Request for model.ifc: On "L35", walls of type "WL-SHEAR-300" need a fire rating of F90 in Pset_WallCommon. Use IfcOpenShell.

First a look at what the model holds.

```python
import ifcopenshell
import ifcopenshell.util.element

model = ifcopenshell.open("model.ifc")
print(model.schema)
storey = next(s for s in model.by_type("IfcBuildingStorey") if s.Name == "L35")
walls = [e for e in ifcopenshell.util.element.get_decomposition(storey) if e.is_a("IfcWall")]
seen = {}
for e in walls:
    element_type = ifcopenshell.util.element.get_type(e)
    key = (element_type.Name if element_type != e and element_type else None, ifcopenshell.util.element.get_pset(e, "Pset_WallCommon", "FireRating"))
    seen[key] = seen.get(key, 0) + 1
for (name, value), count in sorted(seen.items(), key=str):
    print(count, "x", name, "|", value)
```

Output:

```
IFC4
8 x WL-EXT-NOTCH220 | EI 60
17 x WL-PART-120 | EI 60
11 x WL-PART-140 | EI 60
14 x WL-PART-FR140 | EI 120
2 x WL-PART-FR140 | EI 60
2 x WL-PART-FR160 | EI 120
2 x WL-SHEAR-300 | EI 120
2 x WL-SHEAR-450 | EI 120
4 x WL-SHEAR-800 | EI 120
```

```python
import ifcopenshell
import ifcopenshell.api.pset
import ifcopenshell.util.element

model = ifcopenshell.open("model.ifc")

storey = next(s for s in model.by_type("IfcBuildingStorey") if s.Name == "L35")
walls = [e for e in ifcopenshell.util.element.get_decomposition(storey) if e.is_a("IfcWall")]

count = 0
for e in walls:
    element_type = ifcopenshell.util.element.get_type(e)
    if element_type in (None, e) or element_type.Name != "WL-SHEAR-300":
        continue
    # add_pset returns the element's existing set when there is one.
    pset = ifcopenshell.api.pset.add_pset(model, product=e, name="Pset_WallCommon")
    ifcopenshell.api.pset.edit_pset(model, pset=pset, properties={"FireRating": "F90"})
    count += 1

print(count, "walls updated")

model.write("model_rev.ifc")
```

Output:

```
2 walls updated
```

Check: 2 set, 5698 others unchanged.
